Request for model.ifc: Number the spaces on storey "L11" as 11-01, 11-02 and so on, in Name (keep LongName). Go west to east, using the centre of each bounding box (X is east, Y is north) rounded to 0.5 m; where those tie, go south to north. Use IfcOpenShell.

First a look at what the model holds.

```python
import ifcopenshell
import ifcopenshell.util.element
import ifcopenshell.util.placement

model = ifcopenshell.open("model.ifc")
print(model.schema)
storey = next(s for s in model.by_type("IfcBuildingStorey") if s.Name == "L11")
spaces = [e for e in ifcopenshell.util.element.get_decomposition(storey) if e.is_a("IfcSpace")]
for e in sorted(spaces, key=lambda e: e.id()):
    origin = ifcopenshell.util.placement.get_local_placement(e.ObjectPlacement)[:3, 3]
    print(e.id(), e.Name, e.LongName, origin.round(2) + 0.0, sep=" | ")
```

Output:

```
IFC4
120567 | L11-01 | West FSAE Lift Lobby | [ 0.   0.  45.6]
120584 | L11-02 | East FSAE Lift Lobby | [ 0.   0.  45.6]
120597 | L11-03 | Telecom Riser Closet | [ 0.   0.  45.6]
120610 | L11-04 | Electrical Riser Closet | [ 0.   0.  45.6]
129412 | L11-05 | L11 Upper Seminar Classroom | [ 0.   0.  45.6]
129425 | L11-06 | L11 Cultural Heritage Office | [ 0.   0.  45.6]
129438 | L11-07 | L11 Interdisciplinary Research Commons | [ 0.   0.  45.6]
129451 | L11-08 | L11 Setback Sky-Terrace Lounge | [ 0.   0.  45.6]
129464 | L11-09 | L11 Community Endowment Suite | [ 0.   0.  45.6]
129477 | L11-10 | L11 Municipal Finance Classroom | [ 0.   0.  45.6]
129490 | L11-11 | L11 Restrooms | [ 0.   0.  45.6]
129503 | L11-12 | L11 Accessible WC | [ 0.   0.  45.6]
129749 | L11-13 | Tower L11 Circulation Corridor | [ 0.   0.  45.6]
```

```python
import ifcopenshell
import ifcopenshell.geom
import ifcopenshell.util.element
import ifcopenshell.util.shape

model = ifcopenshell.open("model.ifc")
settings = ifcopenshell.geom.settings()
settings.set("use-world-coords", True)


def centre(element):
    shape = ifcopenshell.geom.create_shape(settings, element)
    return ifcopenshell.util.shape.get_bbox_centroid(shape.geometry)


storey = next(s for s in model.by_type("IfcBuildingStorey") if s.Name == "L11")
spaces = [e for e in ifcopenshell.util.element.get_decomposition(storey) if e.is_a("IfcSpace")]

# Insertion points can sit at a corner or the storey origin, so sort by the geometry (in metres).
centres = {e: centre(e) for e in spaces}
spaces.sort(key=lambda e: (round(centres[e][0] / 0.5), centres[e][1]))

for i, e in enumerate(spaces, start=1):
    number = f"11-{i:02d}"
    e.Name = number
    print(e.id(), number)

model.write("model_updated.ifc")
```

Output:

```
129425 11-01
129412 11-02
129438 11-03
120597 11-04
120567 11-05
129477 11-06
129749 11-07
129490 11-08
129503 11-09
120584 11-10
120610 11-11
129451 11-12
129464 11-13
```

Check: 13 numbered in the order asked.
